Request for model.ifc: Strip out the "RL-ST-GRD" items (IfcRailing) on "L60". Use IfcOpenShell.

First a look at what the model holds.

```python
import ifcopenshell
import ifcopenshell.util.element

model = ifcopenshell.open("model.ifc")
print(model.schema)
storey = next(s for s in model.by_type("IfcBuildingStorey") if s.Name == "L60")
railings = [e for e in ifcopenshell.util.element.get_decomposition(storey) if e.is_a("IfcRailing")]
seen = {}
for e in railings:
    element_type = ifcopenshell.util.element.get_type(e)
    name = element_type.Name if element_type not in (None, e) else None
    seen[name] = seen.get(name, 0) + 1
for name, count in sorted(seen.items(), key=str):
    print(count, "x", name)
```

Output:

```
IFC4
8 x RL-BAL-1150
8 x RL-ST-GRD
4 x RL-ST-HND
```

```python
import ifcopenshell
import ifcopenshell.api.root
import ifcopenshell.util.element

model = ifcopenshell.open("model.ifc")

storey = next(s for s in model.by_type("IfcBuildingStorey") if s.Name == "L60")
railings = [e for e in ifcopenshell.util.element.get_decomposition(storey) if e.is_a("IfcRailing")]
targets = [e for e in railings if (t := ifcopenshell.util.element.get_type(e)) not in (None, e) and t.Name == "RL-ST-GRD"]

for e in targets:
    ifcopenshell.api.root.remove_product(model, product=e)
print(len(targets), "removed")

model.write("model-out.ifc")
```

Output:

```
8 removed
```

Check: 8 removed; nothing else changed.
